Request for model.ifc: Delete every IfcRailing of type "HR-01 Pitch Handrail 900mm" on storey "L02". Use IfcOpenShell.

First a look at what the model holds.

```python
import ifcopenshell
import ifcopenshell.util.element

model = ifcopenshell.open("model.ifc")
print(model.schema)
storey = next(s for s in model.by_type("IfcBuildingStorey") if s.Name == "L02")
railings = [e for e in ifcopenshell.util.element.get_decomposition(storey) if e.is_a("IfcRailing")]
seen = {}
for e in railings:
    element_type = ifcopenshell.util.element.get_type(e)
    name = element_type.Name if element_type not in (None, e) else None
    seen[name] = seen.get(name, 0) + 1
for name, count in sorted(seen.items(), key=str):
    print(count, "x", name)
```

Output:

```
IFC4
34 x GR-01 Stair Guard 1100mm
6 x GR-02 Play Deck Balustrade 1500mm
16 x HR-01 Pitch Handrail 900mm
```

```python
import ifcopenshell
import ifcopenshell.api.root
import ifcopenshell.util.element

model = ifcopenshell.open("model.ifc")

storey = next(s for s in model.by_type("IfcBuildingStorey") if s.Name == "L02")
railings = [e for e in ifcopenshell.util.element.get_decomposition(storey) if e.is_a("IfcRailing")]
targets = [e for e in railings if (t := ifcopenshell.util.element.get_type(e)) not in (None, e) and t.Name == "HR-01 Pitch Handrail 900mm"]

for e in targets:
    ifcopenshell.api.root.remove_product(model, product=e)
print(len(targets), "removed")

model.write("model_edited.ifc")
```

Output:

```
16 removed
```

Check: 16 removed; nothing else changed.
